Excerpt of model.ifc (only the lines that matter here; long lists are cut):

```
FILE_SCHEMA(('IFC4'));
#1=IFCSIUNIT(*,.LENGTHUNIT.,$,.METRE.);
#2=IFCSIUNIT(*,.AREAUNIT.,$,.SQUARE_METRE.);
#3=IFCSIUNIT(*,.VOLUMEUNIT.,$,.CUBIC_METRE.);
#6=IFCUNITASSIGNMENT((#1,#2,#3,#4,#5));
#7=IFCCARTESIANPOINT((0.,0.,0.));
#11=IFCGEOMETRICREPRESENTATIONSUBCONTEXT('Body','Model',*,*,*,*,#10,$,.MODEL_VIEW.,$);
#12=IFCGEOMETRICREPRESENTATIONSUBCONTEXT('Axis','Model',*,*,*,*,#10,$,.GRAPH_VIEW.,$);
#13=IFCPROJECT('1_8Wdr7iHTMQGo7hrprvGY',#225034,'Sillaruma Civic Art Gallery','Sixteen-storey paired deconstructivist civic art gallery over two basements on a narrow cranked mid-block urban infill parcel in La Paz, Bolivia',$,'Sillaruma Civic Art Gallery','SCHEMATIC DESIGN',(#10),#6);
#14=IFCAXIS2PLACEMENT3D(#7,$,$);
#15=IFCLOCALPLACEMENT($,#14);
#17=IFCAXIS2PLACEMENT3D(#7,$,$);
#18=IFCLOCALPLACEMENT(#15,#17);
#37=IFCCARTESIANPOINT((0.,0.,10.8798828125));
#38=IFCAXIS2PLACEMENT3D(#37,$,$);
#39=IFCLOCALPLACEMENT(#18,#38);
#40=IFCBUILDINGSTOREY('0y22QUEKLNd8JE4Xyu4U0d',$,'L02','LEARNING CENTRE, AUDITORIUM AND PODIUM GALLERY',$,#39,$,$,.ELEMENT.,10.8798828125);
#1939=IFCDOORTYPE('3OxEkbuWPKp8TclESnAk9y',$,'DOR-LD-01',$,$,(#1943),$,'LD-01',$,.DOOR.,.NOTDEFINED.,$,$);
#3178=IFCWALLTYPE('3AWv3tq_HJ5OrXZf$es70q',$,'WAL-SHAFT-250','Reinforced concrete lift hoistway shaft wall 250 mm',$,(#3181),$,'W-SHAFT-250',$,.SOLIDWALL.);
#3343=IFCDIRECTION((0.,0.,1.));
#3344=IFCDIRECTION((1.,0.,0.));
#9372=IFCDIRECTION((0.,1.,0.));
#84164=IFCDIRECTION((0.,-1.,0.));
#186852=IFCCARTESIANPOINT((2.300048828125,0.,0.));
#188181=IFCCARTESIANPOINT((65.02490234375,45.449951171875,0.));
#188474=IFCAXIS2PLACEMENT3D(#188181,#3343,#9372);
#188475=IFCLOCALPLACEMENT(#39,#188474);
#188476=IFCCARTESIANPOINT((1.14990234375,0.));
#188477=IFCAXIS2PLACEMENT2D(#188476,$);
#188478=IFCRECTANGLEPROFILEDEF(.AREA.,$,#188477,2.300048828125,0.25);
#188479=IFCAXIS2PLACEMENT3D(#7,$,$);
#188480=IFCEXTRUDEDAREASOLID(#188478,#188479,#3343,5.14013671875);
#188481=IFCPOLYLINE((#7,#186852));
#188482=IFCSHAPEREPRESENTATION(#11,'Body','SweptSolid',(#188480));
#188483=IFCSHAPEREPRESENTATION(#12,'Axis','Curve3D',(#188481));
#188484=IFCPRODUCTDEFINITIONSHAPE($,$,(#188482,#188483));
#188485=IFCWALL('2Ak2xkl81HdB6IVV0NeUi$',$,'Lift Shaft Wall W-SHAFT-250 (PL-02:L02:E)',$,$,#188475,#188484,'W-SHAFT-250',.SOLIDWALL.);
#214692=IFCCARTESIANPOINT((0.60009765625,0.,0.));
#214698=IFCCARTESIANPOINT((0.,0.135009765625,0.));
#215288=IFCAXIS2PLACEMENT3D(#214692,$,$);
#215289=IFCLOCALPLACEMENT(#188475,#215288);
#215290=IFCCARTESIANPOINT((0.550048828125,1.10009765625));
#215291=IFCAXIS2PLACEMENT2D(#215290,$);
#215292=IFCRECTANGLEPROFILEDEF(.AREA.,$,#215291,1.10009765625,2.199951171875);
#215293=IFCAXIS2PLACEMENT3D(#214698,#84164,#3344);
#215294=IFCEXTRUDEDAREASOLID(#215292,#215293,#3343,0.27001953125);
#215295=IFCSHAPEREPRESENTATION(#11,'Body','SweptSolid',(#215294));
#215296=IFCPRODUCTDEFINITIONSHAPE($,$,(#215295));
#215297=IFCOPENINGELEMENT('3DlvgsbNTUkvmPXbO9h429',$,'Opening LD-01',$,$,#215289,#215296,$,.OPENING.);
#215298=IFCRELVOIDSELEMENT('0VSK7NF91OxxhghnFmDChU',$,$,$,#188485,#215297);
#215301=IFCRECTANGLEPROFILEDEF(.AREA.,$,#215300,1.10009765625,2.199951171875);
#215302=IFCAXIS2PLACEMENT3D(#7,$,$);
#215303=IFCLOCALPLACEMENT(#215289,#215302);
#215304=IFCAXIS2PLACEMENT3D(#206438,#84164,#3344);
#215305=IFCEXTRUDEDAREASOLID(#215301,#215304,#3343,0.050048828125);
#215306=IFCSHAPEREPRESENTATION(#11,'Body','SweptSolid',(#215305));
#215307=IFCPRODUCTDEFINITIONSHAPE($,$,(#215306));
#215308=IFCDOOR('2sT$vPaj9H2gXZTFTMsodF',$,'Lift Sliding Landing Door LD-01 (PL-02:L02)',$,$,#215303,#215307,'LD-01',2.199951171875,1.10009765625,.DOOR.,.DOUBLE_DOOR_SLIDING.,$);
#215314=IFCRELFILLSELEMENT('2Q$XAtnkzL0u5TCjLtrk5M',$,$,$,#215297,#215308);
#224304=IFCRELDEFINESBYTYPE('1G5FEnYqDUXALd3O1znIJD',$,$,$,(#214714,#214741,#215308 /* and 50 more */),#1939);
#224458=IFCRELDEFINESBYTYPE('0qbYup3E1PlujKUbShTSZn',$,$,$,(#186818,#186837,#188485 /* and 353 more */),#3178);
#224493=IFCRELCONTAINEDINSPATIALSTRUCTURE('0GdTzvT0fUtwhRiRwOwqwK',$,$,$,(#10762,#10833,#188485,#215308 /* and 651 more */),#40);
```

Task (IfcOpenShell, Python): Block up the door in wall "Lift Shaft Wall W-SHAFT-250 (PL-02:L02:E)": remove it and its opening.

```python
import ifcopenshell
import ifcopenshell.api.feature
import ifcopenshell.api.root
import ifcopenshell.geom
import ifcopenshell.util.shape

model = ifcopenshell.open("model.ifc")
settings = ifcopenshell.geom.settings()


def volume(element):
    """Net volume in cubic metres, openings subtracted."""
    shape = ifcopenshell.geom.create_shape(settings, element)
    return ifcopenshell.util.shape.get_volume(shape.geometry)


door = model.by_guid("2sT$vPaj9H2gXZTFTMsodF")
opening = door.FillsVoids[0].RelatingOpeningElement
wall = opening.VoidsElements[0].RelatingBuildingElement
before = volume(wall)

ifcopenshell.api.root.remove_product(model, product=door)
ifcopenshell.api.feature.remove_feature(model, feature=opening)

after = volume(wall)

print(f"wall volume {before:.3f} -> {after:.3f} m3")

model.write("model-out.ifc")
```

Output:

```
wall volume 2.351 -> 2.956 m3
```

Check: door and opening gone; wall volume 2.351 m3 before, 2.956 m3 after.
